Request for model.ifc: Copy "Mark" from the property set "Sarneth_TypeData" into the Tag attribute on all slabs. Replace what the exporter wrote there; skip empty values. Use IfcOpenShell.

First a look at what the model holds.

```python
import ifcopenshell
import ifcopenshell.util.element

model = ifcopenshell.open("model.ifc")
print(model.schema)
slabs = model.by_type("IfcSlab")
print(len(slabs), "slabs")
for e in slabs[:8]:
    source = ifcopenshell.util.element.get_pset(e, "Sarneth_TypeData", "Mark")
    target = e.Tag
    print(e.id(), repr(source), repr(target), sep=" | ")
```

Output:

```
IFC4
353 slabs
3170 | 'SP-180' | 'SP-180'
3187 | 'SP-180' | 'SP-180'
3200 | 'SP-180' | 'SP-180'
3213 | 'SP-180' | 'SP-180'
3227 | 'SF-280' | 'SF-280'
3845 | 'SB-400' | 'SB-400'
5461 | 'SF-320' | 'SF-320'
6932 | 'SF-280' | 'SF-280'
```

```python
import ifcopenshell
import ifcopenshell.util.element

model = ifcopenshell.open("model.ifc")

count = 0
for e in model.by_type("IfcSlab"):
    value = ifcopenshell.util.element.get_pset(e, "Sarneth_TypeData", "Mark")
    current = e.Tag
    if not value or not value.strip() or current == value:
        continue
    e.Tag = value
    count += 1

print(count, "slabs updated")

model.write("model_v2.ifc")
```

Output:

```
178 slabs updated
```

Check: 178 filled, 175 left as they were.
